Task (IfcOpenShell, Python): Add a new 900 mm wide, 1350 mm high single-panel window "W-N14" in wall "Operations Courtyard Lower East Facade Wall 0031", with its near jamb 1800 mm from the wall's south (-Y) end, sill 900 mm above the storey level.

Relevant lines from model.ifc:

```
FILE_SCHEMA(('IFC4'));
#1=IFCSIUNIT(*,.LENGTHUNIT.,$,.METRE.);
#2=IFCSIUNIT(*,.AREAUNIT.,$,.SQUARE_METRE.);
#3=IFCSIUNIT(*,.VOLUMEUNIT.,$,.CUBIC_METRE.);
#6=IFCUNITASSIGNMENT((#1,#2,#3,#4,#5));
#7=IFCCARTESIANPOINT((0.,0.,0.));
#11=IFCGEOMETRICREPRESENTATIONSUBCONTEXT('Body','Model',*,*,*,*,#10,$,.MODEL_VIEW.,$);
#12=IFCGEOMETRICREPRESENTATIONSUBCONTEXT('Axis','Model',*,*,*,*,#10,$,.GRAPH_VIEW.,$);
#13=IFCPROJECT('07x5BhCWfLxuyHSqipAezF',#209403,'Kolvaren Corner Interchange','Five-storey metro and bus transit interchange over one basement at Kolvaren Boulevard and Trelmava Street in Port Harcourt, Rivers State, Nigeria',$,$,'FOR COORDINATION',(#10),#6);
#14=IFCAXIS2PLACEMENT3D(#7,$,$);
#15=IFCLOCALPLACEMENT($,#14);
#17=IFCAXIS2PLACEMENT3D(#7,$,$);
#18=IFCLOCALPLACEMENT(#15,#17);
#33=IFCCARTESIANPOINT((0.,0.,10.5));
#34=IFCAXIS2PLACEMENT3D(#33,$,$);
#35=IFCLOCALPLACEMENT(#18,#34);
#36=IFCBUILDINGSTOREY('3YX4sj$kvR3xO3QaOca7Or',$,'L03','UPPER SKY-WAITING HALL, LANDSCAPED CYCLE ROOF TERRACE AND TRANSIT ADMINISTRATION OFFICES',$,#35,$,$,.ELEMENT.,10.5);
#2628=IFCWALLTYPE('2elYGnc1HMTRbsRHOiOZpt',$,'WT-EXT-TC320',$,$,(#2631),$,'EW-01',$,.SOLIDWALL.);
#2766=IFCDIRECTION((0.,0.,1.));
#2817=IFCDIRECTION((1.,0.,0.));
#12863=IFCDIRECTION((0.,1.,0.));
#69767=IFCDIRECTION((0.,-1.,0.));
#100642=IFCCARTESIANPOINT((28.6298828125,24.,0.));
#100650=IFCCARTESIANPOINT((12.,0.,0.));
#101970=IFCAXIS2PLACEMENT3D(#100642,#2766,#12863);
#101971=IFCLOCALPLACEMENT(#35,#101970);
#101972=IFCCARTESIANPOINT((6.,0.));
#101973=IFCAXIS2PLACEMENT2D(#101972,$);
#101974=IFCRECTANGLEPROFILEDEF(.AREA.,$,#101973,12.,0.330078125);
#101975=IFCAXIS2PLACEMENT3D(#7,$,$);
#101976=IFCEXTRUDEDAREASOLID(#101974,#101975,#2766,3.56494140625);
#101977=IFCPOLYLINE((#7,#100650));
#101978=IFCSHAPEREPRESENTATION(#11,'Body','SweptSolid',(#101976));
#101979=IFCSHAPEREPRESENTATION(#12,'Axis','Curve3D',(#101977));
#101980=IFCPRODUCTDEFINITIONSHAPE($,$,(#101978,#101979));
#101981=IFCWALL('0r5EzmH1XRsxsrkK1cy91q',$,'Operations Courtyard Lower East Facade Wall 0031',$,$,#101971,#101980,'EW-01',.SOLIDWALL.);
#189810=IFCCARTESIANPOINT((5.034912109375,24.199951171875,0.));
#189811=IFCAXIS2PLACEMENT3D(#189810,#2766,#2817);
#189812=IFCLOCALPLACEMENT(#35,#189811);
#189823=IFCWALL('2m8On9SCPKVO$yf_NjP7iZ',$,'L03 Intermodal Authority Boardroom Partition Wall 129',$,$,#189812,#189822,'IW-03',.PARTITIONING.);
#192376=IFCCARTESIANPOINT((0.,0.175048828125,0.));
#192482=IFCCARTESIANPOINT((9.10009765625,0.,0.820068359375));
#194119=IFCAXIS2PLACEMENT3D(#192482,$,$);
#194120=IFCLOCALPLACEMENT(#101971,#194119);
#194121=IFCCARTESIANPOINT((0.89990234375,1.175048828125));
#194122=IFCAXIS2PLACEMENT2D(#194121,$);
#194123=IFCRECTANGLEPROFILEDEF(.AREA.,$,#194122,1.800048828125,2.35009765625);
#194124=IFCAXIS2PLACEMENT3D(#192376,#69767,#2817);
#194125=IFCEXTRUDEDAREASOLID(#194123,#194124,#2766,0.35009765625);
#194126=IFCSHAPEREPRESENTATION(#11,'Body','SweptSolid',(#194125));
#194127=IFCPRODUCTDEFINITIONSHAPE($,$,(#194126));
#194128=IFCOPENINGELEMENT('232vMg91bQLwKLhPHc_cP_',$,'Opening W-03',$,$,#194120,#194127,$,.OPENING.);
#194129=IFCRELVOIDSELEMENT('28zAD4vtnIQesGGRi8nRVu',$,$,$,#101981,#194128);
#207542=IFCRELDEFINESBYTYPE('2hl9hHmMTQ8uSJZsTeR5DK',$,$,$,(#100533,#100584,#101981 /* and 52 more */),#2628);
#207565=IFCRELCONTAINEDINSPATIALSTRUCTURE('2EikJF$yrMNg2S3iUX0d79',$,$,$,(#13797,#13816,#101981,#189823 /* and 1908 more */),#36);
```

```python
import numpy as np
import ifcopenshell
import ifcopenshell.api.feature
import ifcopenshell.api.geometry
import ifcopenshell.api.root
import ifcopenshell.api.spatial
import ifcopenshell.geom
import ifcopenshell.util.element
import ifcopenshell.util.placement
import ifcopenshell.util.representation
import ifcopenshell.util.shape
import ifcopenshell.util.unit

model = ifcopenshell.open("model.ifc")
unit_scale = ifcopenshell.util.unit.calculate_unit_scale(model)
settings = ifcopenshell.geom.settings()


def volume(element):
    """Net volume in cubic metres, openings subtracted."""
    shape = ifcopenshell.geom.create_shape(settings, element)
    return ifcopenshell.util.shape.get_volume(shape.geometry)


wall = model.by_id(101981)
storey = ifcopenshell.util.element.get_container(wall, ifc_class="IfcBuildingStorey")
context = ifcopenshell.util.representation.get_context(model, "Model", "Body", "MODEL_VIEW")
before = volume(wall)

width, height, from_end, sill = 0.9, 1.35, 1.8, 0.9  # metres

# The wall runs along its own X axis, and the end named is its -X end.
wall_shape = ifcopenshell.geom.create_shape(settings, wall)
x, y, z = ifcopenshell.util.shape.get_vertices(wall_shape.geometry).T
start = x.min() + from_end
face, thickness = float(y.min()), float(y.max() - y.min())
wall_matrix = ifcopenshell.util.placement.get_local_placement(wall.ObjectPlacement)
level = ifcopenshell.util.placement.get_local_placement(storey.ObjectPlacement)[2, 3]


def in_wall(x, y):
    """Placement at x, y metres in the wall's axes, at sill height."""
    matrix = wall_matrix.copy()
    matrix[:, 3] = wall_matrix @ np.array([x / unit_scale, y / unit_scale, 0.0, 1.0])
    matrix[2, 3] = level + sill / unit_scale
    return matrix


# Opening: a box that overshoots both wall faces by 50 mm.
opening = ifcopenshell.api.root.create_entity(model, ifc_class="IfcOpeningElement", predefined_type="OPENING")
box = ifcopenshell.api.geometry.add_wall_representation(
    model, context=context, length=width, height=height, thickness=thickness + 0.1
)
ifcopenshell.api.geometry.assign_representation(model, product=opening, representation=box)
ifcopenshell.api.geometry.edit_object_placement(model, product=opening, matrix=in_wall(start, face - 0.05), is_si=False)
ifcopenshell.api.feature.add_feature(model, feature=opening, element=wall)

window = ifcopenshell.api.root.create_entity(model, ifc_class="IfcWindow", name="W-N14", predefined_type="WINDOW")
window.OverallWidth, window.OverallHeight = width / unit_scale, height / unit_scale
window.PartitioningType = "SINGLE_PANEL"
body = ifcopenshell.api.geometry.add_window_representation(
    model,
    context=context,
    overall_width=window.OverallWidth,
    overall_height=window.OverallHeight,
    partition_type="SINGLE_PANEL",
)
ifcopenshell.api.geometry.assign_representation(model, product=window, representation=body)
ifcopenshell.api.spatial.assign_container(model, products=[window], relating_structure=storey)
ifcopenshell.api.feature.add_filling(model, opening=opening, element=window)

# Centre the window in the wall's thickness.
ifcopenshell.api.geometry.edit_object_placement(model, product=window, matrix=in_wall(start, face), is_si=False)
window_shape = ifcopenshell.geom.create_shape(settings, window)
depth = ifcopenshell.util.shape.get_vertices(window_shape.geometry)[:, 1]
offset = face + thickness / 2 - (depth.min() + depth.max()) / 2
ifcopenshell.api.geometry.edit_object_placement(model, product=window, matrix=in_wall(start, offset), is_si=False)

after = volume(wall)

print(f"wall volume {before:.3f} -> {after:.3f} m3")

model.write("model_edited.ifc")
```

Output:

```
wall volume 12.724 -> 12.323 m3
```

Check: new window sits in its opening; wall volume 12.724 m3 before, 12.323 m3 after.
